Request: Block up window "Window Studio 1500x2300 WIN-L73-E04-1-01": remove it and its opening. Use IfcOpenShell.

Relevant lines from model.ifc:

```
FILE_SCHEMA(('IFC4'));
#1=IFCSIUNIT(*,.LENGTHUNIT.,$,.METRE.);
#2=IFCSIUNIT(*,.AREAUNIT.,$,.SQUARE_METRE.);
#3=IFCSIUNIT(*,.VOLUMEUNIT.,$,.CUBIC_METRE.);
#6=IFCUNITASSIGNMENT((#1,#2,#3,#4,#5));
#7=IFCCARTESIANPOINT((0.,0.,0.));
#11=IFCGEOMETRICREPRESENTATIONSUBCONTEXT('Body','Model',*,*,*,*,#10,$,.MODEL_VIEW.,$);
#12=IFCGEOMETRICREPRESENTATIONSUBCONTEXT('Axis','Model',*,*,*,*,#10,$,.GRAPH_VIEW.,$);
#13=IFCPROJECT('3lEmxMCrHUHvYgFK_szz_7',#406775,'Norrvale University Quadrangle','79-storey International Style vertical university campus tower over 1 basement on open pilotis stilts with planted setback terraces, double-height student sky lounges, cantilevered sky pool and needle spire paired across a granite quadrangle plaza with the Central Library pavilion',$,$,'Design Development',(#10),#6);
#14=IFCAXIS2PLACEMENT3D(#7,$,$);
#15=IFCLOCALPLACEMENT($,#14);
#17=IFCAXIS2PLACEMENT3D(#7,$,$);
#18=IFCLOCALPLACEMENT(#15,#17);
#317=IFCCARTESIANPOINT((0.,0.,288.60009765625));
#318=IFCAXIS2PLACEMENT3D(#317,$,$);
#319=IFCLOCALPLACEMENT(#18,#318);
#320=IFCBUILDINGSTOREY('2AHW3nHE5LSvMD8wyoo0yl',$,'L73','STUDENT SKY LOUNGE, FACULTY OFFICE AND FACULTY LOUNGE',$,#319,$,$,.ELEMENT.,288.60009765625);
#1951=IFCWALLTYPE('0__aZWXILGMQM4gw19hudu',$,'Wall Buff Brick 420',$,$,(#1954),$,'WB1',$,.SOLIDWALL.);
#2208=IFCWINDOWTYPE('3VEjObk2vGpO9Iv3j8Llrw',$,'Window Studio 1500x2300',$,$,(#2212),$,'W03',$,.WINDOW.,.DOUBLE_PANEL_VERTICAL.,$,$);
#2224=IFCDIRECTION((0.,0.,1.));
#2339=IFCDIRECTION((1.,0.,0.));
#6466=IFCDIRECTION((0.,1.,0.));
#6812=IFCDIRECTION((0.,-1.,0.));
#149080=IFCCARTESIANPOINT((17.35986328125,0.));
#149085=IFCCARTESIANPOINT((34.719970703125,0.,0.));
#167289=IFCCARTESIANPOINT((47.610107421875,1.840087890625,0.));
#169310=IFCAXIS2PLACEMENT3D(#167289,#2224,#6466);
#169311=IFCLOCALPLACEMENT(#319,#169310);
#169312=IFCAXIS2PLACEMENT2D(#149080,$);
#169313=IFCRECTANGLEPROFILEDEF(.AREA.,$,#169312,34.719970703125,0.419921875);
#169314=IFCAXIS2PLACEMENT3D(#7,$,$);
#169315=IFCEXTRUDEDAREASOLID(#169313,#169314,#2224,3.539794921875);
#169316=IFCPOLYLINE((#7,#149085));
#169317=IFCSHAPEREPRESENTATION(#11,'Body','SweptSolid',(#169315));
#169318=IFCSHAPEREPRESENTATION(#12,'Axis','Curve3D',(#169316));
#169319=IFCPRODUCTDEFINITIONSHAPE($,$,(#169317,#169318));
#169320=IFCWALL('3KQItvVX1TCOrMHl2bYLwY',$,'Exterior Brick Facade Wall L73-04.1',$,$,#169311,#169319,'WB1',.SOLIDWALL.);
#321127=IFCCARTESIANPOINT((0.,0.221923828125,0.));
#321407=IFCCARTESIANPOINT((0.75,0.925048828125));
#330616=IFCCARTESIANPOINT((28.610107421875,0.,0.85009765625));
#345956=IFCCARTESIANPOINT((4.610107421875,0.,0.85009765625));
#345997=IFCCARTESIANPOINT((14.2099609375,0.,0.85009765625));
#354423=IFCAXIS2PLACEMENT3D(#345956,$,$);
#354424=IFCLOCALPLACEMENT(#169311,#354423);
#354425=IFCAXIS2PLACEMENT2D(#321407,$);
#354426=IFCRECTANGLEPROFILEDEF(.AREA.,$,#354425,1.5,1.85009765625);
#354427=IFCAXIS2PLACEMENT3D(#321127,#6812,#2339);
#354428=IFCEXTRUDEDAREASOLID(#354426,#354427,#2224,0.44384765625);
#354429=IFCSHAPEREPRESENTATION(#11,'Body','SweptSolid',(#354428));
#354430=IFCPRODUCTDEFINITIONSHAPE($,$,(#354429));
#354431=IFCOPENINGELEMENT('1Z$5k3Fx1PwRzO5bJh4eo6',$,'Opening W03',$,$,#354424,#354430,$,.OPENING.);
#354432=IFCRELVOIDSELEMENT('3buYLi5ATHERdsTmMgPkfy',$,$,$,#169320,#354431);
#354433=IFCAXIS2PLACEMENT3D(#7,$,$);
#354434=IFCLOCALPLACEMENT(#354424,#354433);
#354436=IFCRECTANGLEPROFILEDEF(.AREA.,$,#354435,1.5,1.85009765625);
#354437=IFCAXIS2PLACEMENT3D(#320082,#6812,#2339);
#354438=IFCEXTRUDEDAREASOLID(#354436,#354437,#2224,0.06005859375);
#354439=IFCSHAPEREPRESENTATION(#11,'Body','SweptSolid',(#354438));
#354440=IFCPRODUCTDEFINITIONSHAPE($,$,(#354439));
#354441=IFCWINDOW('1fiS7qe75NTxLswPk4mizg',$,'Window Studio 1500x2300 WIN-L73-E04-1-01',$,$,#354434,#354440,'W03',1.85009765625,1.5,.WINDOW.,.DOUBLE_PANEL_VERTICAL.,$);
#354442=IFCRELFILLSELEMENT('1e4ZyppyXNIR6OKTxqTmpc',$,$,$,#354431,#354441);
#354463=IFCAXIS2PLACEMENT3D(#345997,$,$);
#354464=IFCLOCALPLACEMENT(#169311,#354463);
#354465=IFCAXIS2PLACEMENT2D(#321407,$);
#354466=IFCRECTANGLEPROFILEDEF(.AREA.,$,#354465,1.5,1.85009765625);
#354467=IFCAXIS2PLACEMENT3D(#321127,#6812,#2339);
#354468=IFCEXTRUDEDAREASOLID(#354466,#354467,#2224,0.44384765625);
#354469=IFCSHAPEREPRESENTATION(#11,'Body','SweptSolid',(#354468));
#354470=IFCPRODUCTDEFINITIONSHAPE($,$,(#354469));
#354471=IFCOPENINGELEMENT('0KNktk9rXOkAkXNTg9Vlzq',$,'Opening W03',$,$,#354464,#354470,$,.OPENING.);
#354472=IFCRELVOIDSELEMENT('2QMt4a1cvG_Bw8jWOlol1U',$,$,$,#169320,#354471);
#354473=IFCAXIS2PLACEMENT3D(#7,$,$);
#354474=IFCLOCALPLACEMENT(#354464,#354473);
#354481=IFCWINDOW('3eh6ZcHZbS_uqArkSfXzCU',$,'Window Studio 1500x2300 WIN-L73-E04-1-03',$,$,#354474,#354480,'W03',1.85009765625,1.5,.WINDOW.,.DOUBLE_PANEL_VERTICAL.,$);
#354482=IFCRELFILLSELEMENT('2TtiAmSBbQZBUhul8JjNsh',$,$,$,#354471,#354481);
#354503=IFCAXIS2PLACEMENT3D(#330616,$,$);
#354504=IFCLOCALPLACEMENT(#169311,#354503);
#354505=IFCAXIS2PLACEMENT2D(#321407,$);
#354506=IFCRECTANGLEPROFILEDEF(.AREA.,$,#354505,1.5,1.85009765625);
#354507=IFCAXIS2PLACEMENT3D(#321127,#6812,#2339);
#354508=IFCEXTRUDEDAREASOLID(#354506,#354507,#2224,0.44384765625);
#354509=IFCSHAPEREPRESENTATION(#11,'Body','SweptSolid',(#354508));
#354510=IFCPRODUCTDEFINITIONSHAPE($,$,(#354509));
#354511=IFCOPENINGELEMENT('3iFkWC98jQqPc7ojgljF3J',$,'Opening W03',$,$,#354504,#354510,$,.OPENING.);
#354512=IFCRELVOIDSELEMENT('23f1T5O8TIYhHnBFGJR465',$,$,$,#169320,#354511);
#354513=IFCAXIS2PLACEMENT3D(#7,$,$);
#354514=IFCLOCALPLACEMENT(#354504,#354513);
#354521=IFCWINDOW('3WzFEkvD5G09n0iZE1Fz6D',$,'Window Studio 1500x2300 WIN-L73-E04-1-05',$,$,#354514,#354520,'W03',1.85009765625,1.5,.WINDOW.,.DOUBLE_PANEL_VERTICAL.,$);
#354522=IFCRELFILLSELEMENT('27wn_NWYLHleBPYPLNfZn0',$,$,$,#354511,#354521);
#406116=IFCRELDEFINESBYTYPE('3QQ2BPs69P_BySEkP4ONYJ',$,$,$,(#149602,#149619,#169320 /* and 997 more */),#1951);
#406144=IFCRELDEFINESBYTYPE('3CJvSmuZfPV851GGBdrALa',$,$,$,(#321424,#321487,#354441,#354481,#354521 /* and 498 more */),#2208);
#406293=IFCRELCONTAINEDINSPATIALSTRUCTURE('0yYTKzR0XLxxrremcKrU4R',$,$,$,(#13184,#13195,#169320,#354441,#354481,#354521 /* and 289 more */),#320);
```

```python
import ifcopenshell
import ifcopenshell.api.feature
import ifcopenshell.api.root
import ifcopenshell.geom
import ifcopenshell.util.shape

model = ifcopenshell.open("model.ifc")
settings = ifcopenshell.geom.settings()


def volume(element):
    """Net volume in cubic metres, openings subtracted."""
    shape = ifcopenshell.geom.create_shape(settings, element)
    return ifcopenshell.util.shape.get_volume(shape.geometry)


window = model.by_id(354441)
opening = window.FillsVoids[0].RelatingOpeningElement
wall = opening.VoidsElements[0].RelatingBuildingElement
before = volume(wall)

ifcopenshell.api.root.remove_product(model, product=window)
ifcopenshell.api.feature.remove_feature(model, feature=opening)

after = volume(wall)

print(f"wall volume {before:.3f} -> {after:.3f} m3")

model.write("model_v2.ifc")
```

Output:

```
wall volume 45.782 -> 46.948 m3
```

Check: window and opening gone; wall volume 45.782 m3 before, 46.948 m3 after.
